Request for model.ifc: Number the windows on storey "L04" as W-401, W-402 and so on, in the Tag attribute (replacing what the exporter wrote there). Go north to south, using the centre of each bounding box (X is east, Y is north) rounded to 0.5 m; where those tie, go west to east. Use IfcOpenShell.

First a look at what the model holds.

```python
import ifcopenshell
import ifcopenshell.util.element
import ifcopenshell.util.placement

model = ifcopenshell.open("model.ifc")
print(model.schema)
storey = next(s for s in model.by_type("IfcBuildingStorey") if s.Name == "L04")
windows = [e for e in ifcopenshell.util.element.get_decomposition(storey) if e.is_a("IfcWindow")]
for e in sorted(windows, key=lambda e: e.id()):
    origin = ifcopenshell.util.placement.get_local_placement(e.ObjectPlacement)[:3, 3]
    print(e.id(), e.Tag, e.Name, origin.round(2) + 0.0, sep=" | ")
```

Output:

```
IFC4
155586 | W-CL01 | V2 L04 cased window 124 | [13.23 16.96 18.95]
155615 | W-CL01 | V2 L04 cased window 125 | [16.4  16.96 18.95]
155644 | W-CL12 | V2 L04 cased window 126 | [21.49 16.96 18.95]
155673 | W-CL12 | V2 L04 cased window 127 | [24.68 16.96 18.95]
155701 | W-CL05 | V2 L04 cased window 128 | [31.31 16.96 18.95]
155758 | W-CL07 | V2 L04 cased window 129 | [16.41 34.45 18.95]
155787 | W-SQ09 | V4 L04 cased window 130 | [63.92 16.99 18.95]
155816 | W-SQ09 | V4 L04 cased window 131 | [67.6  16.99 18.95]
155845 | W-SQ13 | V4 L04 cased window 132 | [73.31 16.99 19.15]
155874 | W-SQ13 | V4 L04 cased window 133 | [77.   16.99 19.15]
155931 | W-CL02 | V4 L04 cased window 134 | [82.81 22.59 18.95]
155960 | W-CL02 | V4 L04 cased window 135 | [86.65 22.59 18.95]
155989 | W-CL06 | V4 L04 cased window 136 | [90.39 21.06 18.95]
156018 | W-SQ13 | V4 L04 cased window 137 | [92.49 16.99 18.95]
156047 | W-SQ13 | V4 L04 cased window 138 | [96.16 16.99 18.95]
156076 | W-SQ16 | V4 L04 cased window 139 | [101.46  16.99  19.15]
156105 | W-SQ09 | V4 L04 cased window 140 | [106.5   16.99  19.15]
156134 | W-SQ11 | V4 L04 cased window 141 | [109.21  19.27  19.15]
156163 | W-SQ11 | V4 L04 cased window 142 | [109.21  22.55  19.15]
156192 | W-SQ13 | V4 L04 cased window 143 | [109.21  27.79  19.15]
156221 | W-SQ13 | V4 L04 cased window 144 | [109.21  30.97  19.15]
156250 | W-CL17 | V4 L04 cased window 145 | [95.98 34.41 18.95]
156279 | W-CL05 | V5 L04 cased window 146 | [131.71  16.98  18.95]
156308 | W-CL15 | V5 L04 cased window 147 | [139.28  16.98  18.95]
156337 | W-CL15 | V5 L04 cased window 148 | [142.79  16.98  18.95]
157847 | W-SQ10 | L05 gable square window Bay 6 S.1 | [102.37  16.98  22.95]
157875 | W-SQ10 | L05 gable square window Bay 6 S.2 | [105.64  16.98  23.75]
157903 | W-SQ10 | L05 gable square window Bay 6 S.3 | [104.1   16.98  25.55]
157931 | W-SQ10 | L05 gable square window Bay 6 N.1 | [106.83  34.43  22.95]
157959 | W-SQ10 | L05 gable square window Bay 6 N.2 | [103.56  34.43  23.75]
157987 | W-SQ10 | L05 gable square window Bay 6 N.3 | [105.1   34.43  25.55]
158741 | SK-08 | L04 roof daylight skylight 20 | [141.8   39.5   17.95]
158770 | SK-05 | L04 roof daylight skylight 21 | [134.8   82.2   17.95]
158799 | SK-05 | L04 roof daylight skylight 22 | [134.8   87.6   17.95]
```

```python
import ifcopenshell
import ifcopenshell.geom
import ifcopenshell.util.element
import ifcopenshell.util.shape

model = ifcopenshell.open("model.ifc")
settings = ifcopenshell.geom.settings()
settings.set("use-world-coords", True)


def centre(element):
    shape = ifcopenshell.geom.create_shape(settings, element)
    return ifcopenshell.util.shape.get_bbox_centroid(shape.geometry)


storey = next(s for s in model.by_type("IfcBuildingStorey") if s.Name == "L04")
windows = [e for e in ifcopenshell.util.element.get_decomposition(storey) if e.is_a("IfcWindow")]

# Insertion points can sit at a corner or the storey origin, so sort by the geometry (in metres).
centres = {e: centre(e) for e in windows}
windows.sort(key=lambda e: (-round(centres[e][1] / 0.5), centres[e][0]))

for i, e in enumerate(windows, start=1):
    number = f"W-4{i:02d}"
    e.Tag = number
    print(e.id(), number)

model.write("model_v2.ifc")
```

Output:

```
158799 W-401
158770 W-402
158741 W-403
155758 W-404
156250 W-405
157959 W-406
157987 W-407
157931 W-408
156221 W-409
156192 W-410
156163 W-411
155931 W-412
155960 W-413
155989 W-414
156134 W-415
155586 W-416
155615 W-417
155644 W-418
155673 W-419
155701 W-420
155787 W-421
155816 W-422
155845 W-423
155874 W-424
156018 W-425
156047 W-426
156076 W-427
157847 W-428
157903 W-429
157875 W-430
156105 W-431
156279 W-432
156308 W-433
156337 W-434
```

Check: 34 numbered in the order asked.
